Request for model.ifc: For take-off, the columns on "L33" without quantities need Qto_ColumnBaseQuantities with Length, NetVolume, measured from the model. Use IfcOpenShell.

First a look at what the model holds.

```python
import ifcopenshell
import ifcopenshell.util.element
import ifcopenshell.util.unit

model = ifcopenshell.open("model.ifc")
print(model.schema)
for unit_type in ("LENGTHUNIT", "AREAUNIT", "VOLUMEUNIT"):
    print(unit_type, ifcopenshell.util.unit.calculate_unit_scale(model, unit_type))
storey = next(s for s in model.by_type("IfcBuildingStorey") if s.Name == "L33")
columns = [e for e in ifcopenshell.util.element.get_decomposition(storey) if e.is_a("IfcColumn")]
for e in sorted(columns, key=lambda e: e.id()):
    print(e.id(), e.is_a(), e.Name, list(ifcopenshell.util.element.get_psets(e, qtos_only=True)), sep=" | ")
```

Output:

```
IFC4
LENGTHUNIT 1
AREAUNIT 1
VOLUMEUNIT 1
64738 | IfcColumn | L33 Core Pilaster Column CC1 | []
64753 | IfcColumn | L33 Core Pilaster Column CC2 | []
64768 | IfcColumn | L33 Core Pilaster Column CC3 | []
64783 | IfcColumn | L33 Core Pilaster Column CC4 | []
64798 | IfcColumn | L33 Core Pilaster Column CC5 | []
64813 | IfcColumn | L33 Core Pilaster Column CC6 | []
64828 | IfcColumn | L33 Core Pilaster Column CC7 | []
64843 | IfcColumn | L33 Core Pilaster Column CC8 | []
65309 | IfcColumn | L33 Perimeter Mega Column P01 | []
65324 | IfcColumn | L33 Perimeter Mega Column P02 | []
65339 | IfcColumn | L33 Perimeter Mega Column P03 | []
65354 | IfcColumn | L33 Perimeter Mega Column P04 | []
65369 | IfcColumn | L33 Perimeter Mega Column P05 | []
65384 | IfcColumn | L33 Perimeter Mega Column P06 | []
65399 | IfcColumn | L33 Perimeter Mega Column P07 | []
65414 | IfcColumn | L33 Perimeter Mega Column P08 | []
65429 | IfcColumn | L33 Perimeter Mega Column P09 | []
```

```python
import ifcopenshell
import ifcopenshell.api.pset
import ifcopenshell.geom
import ifcopenshell.util.element
import ifcopenshell.util.shape
import ifcopenshell.util.unit

model = ifcopenshell.open("model.ifc")
unit_scale = ifcopenshell.util.unit.calculate_unit_scale(model)
volume_scale = ifcopenshell.util.unit.calculate_unit_scale(model, "VOLUMEUNIT")
settings = ifcopenshell.geom.settings()

storey = next(s for s in model.by_type("IfcBuildingStorey") if s.Name == "L33")
columns = [e for e in ifcopenshell.util.element.get_decomposition(storey) if e.is_a("IfcColumn")]

for e in sorted(columns, key=lambda e: e.id()):
    if ifcopenshell.util.element.get_psets(e, qtos_only=True, should_inherit=False):
        continue
    # Geometry comes back in metres, in the element's own axes.
    shape = ifcopenshell.geom.create_shape(settings, e)
    values = {
        "Length": ifcopenshell.util.shape.get_z(shape.geometry) / unit_scale,
        "NetVolume": ifcopenshell.util.shape.get_volume(shape.geometry) / volume_scale,
    }
    qto = ifcopenshell.api.pset.add_qto(model, product=e, name="Qto_ColumnBaseQuantities")
    ifcopenshell.api.pset.edit_qto(model, qto=qto, properties=values)
    print(e.id(), {k: round(v, 3) for k, v in values.items()})

model.write("model_edited.ifc")
```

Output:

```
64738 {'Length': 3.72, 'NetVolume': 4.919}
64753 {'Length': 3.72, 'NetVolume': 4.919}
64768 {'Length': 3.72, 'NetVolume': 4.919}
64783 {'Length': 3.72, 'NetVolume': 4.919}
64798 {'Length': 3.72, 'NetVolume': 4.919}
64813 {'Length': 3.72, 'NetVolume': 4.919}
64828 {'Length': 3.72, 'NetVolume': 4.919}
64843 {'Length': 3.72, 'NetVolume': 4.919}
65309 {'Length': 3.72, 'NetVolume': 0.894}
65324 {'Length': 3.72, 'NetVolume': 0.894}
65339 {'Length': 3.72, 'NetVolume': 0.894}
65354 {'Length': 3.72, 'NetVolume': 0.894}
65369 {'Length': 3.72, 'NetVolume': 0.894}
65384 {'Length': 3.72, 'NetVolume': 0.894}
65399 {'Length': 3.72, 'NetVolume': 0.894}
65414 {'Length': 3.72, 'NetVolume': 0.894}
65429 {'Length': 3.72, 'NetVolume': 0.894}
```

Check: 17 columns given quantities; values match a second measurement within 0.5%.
